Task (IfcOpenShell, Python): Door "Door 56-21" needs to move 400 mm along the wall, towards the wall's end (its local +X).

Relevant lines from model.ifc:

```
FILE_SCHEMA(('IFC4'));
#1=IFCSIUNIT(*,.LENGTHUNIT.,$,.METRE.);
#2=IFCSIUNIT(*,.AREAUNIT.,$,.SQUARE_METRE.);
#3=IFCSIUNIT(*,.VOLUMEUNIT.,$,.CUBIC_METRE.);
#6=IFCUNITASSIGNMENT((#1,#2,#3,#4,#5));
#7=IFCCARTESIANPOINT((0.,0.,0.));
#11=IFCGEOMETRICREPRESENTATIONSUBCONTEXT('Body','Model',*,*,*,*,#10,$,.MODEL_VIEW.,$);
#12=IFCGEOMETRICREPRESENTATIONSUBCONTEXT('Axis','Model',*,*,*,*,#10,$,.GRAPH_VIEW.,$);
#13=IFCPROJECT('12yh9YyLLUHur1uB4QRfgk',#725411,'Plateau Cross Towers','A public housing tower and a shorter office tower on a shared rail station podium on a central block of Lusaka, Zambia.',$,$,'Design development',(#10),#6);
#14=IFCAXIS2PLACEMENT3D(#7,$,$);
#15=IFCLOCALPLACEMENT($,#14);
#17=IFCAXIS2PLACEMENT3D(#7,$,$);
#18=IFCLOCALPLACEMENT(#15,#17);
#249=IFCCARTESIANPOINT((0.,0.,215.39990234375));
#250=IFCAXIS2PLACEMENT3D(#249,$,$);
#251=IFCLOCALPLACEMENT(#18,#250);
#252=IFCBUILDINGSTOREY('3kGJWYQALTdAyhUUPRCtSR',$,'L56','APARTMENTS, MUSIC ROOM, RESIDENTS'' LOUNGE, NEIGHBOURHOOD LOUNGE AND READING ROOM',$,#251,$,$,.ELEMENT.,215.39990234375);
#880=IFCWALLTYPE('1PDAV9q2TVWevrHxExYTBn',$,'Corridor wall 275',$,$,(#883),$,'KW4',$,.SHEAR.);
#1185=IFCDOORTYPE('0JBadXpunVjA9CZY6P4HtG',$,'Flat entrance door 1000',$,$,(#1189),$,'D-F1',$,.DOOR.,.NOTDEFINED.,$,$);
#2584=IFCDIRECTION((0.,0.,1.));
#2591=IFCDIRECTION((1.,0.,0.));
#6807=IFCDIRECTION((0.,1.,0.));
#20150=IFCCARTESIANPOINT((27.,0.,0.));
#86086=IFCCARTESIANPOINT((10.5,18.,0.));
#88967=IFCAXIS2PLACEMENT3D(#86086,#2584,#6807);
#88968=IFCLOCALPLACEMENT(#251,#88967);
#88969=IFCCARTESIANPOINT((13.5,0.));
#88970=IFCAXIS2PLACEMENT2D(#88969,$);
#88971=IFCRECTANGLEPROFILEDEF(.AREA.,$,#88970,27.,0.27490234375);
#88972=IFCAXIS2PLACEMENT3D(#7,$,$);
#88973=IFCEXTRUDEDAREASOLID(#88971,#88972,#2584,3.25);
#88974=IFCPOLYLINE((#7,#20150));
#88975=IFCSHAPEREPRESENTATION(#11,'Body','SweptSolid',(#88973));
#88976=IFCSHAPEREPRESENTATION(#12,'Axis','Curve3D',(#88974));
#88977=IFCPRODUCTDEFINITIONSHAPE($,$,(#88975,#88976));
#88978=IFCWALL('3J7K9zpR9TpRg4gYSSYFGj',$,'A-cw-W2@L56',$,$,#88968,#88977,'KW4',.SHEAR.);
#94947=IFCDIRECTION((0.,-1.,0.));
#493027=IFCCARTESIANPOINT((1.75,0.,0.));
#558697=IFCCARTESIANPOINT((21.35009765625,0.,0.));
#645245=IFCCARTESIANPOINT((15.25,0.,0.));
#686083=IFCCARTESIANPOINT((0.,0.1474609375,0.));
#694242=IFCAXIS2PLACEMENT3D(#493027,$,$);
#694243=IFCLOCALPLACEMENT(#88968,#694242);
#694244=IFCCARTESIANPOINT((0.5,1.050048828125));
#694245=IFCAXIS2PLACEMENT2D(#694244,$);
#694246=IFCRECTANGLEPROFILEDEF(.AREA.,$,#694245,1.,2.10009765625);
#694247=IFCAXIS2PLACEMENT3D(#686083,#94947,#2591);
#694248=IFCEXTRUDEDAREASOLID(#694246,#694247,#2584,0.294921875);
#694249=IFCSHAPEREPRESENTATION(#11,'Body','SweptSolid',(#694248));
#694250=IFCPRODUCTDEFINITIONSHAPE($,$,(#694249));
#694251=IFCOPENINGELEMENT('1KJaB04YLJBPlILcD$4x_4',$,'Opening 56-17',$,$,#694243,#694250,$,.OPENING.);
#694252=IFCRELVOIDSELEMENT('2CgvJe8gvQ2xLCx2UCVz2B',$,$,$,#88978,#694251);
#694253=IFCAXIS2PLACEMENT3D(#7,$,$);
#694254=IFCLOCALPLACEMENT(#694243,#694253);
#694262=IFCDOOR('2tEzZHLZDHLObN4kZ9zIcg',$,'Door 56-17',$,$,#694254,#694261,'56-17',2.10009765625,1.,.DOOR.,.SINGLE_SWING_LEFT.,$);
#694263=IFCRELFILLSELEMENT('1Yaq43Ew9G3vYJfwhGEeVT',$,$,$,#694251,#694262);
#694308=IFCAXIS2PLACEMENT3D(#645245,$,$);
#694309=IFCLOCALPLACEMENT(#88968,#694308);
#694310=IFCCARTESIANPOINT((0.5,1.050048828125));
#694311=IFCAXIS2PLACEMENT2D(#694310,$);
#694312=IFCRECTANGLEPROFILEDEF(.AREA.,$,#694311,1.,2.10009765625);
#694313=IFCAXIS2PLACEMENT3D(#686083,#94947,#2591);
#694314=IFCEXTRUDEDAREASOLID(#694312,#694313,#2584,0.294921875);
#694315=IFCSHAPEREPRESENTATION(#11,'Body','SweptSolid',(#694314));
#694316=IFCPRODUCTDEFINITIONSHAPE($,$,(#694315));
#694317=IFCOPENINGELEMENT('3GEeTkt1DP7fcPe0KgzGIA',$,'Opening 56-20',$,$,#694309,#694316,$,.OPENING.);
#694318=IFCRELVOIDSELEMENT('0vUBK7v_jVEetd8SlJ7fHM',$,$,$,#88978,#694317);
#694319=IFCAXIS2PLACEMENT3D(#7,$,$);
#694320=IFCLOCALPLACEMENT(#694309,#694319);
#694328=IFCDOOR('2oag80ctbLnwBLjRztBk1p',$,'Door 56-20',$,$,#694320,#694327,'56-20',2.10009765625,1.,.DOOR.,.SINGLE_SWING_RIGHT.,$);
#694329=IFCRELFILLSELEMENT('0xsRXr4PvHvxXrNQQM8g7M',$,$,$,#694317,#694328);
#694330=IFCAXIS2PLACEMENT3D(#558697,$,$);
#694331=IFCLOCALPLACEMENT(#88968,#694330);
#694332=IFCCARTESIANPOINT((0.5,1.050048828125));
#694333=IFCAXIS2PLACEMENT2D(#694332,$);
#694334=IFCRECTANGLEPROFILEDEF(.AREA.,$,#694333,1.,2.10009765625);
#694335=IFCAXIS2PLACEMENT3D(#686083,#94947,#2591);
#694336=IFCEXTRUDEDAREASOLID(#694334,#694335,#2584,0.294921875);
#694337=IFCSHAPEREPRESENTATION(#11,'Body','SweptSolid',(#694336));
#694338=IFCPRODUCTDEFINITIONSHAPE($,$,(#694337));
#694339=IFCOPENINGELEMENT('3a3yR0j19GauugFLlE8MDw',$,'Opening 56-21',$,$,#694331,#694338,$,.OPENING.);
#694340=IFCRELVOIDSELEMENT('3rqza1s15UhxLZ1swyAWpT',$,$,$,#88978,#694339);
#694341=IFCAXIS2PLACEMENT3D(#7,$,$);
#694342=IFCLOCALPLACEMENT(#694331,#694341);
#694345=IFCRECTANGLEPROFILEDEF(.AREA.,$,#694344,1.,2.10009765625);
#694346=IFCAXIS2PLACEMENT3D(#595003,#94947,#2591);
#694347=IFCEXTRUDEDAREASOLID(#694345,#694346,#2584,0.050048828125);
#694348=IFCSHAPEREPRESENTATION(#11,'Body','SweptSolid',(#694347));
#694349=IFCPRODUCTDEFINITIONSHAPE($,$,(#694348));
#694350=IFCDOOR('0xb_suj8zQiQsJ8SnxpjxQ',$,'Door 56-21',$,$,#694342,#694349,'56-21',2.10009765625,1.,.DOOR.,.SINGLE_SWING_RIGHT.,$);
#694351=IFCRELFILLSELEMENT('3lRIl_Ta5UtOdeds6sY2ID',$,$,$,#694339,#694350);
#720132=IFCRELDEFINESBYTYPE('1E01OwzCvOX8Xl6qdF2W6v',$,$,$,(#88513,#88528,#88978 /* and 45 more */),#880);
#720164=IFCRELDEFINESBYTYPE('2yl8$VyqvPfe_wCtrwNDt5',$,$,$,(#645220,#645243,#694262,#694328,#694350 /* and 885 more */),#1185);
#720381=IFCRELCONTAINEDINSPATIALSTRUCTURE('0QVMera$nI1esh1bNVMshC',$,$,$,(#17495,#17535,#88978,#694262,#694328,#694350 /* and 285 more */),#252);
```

```python
import ifcopenshell
import ifcopenshell.api.geometry
import ifcopenshell.util.placement
import ifcopenshell.util.unit

model = ifcopenshell.open("model.ifc")
unit_scale = ifcopenshell.util.unit.calculate_unit_scale(model)

door = model.by_guid("0xb_suj8zQiQsJ8SnxpjxQ")
opening = door.FillsVoids[0].RelatingOpeningElement
wall = opening.VoidsElements[0].RelatingBuildingElement

wall_matrix = ifcopenshell.util.placement.get_local_placement(wall.ObjectPlacement)
shift = wall_matrix[:3, 0] * 0.4 / unit_scale
before = ifcopenshell.util.placement.get_local_placement(door.ObjectPlacement)[:3, 3].copy()

# The door is placed relative to its opening, so it follows when the opening moves.
matrix = ifcopenshell.util.placement.get_local_placement(opening.ObjectPlacement)
matrix[:3, 3] += shift
ifcopenshell.api.geometry.edit_object_placement(
    model, product=opening, matrix=matrix, is_si=False, should_transform_children=True
)

after = ifcopenshell.util.placement.get_local_placement(door.ObjectPlacement)[:3, 3]
print("door moved by", (after - before).round(3) + 0.0)

model.write("model_edited.ifc")
```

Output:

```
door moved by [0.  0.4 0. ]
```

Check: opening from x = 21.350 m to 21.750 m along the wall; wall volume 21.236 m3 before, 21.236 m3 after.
